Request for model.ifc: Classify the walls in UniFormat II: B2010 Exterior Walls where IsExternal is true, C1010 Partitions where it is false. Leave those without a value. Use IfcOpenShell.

First a look at what the model holds.

```python
import ifcopenshell
import ifcopenshell.util.element

model = ifcopenshell.open("model.ifc")
print(model.schema)
print("classifications:", [c.Name for c in model.by_type("IfcClassification")])
values = [ifcopenshell.util.element.get_pset(e, "Pset_WallCommon", "IsExternal") for e in model.by_type("IfcWall")]
for value in (True, False, None):
    print("IsExternal", value, values.count(value))
```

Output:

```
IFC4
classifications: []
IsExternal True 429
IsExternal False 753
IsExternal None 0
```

```python
import ifcopenshell
import ifcopenshell.api.classification
import ifcopenshell.util.element

model = ifcopenshell.open("model.ifc")

system = ifcopenshell.api.classification.add_classification(model, classification="UniFormat II")

walls = model.by_type("IfcWall")
external = {e: ifcopenshell.util.element.get_pset(e, "Pset_WallCommon", "IsExternal") for e in walls}
for flag, code, name in ((True, "B2010", "Exterior Walls"), (False, "C1010", "Partitions")):
    products = [e for e in walls if external[e] is flag]
    ifcopenshell.api.classification.add_reference(
        model, products=products, classification=system, identification=code, name=name
    )
    print(code, len(products))

model.write("model_updated.ifc")
```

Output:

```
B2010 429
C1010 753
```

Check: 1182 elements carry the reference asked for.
